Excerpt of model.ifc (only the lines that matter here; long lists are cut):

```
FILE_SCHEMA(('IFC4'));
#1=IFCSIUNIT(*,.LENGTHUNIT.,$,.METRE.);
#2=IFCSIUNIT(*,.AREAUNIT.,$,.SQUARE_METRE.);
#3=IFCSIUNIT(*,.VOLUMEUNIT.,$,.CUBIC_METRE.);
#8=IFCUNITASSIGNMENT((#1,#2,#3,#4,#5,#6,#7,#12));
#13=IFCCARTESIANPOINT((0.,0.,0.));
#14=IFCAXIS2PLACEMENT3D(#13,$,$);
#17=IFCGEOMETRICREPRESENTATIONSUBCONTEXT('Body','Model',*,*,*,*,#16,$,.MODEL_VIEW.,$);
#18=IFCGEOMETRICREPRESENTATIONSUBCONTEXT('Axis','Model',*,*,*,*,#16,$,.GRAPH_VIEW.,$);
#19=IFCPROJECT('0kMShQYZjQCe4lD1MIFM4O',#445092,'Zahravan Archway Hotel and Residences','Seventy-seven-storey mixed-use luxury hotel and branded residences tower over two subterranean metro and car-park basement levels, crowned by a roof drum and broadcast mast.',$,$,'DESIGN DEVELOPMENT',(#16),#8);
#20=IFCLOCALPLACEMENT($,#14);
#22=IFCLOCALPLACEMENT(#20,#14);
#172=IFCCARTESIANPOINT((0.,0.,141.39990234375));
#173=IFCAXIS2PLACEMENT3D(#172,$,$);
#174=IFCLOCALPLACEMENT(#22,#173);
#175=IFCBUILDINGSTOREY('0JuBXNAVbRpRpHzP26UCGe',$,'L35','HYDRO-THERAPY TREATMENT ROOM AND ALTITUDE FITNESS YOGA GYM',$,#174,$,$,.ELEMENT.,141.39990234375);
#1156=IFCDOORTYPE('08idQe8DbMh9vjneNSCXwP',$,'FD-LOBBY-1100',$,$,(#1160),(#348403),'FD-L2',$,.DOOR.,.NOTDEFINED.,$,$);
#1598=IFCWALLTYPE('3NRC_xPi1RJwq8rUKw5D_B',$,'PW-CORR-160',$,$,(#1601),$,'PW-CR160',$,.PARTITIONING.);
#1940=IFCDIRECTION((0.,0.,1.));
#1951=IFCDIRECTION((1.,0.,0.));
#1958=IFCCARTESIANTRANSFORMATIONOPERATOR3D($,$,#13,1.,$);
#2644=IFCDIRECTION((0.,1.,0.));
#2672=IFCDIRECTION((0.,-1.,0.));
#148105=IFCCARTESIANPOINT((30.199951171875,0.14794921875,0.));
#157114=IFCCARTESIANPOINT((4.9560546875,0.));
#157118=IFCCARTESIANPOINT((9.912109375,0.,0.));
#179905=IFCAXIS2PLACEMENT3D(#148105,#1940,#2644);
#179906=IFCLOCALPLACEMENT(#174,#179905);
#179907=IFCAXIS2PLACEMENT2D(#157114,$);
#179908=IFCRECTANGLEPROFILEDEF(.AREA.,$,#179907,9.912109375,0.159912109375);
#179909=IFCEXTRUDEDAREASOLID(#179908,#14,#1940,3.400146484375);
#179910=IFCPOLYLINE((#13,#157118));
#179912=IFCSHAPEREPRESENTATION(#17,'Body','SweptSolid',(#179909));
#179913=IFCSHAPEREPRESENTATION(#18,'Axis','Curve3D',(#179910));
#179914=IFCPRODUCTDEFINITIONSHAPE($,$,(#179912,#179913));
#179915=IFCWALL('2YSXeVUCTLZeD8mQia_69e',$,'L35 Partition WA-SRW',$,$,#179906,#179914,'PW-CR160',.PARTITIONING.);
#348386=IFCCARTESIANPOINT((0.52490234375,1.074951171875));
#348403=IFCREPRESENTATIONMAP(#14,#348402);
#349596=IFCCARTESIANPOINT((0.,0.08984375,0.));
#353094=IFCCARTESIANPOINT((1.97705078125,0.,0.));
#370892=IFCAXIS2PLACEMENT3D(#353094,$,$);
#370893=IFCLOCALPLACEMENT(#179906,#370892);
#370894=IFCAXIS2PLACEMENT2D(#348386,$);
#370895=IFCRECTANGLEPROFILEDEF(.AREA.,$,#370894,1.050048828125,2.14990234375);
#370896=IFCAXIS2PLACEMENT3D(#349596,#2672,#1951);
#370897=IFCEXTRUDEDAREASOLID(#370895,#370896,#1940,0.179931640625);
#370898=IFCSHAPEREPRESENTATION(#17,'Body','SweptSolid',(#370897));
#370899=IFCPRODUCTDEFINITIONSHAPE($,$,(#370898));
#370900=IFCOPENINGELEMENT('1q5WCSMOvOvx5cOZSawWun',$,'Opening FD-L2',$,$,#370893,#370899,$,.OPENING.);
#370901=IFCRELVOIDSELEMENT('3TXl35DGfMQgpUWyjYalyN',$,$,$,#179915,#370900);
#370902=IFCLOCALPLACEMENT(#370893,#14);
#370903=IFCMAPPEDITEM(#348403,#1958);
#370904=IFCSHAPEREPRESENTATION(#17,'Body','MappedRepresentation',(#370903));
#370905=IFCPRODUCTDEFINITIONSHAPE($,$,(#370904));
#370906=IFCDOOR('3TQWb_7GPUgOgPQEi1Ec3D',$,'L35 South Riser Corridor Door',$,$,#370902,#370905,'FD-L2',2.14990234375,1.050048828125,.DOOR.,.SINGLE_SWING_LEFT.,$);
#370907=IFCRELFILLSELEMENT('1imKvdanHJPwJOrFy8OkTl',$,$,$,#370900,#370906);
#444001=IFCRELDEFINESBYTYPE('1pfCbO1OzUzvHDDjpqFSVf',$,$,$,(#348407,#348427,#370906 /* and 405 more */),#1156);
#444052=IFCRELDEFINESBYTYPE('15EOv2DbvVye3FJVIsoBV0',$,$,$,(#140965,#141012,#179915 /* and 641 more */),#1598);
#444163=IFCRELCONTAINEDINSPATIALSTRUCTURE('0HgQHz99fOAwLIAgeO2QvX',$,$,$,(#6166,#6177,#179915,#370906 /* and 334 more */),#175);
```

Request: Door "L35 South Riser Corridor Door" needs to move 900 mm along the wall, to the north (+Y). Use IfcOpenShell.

```python
import ifcopenshell
import ifcopenshell.api.geometry
import ifcopenshell.util.placement
import ifcopenshell.util.unit

model = ifcopenshell.open("model.ifc")
unit_scale = ifcopenshell.util.unit.calculate_unit_scale(model)

door = model.by_guid("3TQWb_7GPUgOgPQEi1Ec3D")
opening = door.FillsVoids[0].RelatingOpeningElement
wall = opening.VoidsElements[0].RelatingBuildingElement

wall_matrix = ifcopenshell.util.placement.get_local_placement(wall.ObjectPlacement)
shift = wall_matrix[:3, 0] * 0.9 / unit_scale
before = ifcopenshell.util.placement.get_local_placement(door.ObjectPlacement)[:3, 3].copy()

# The door is placed relative to its opening, so it follows when the opening moves.
matrix = ifcopenshell.util.placement.get_local_placement(opening.ObjectPlacement)
matrix[:3, 3] += shift
ifcopenshell.api.geometry.edit_object_placement(
    model, product=opening, matrix=matrix, is_si=False, should_transform_children=True
)

after = ifcopenshell.util.placement.get_local_placement(door.ObjectPlacement)[:3, 3]
print("door moved by", (after - before).round(3) + 0.0)

model.write("model_rev.ifc")
```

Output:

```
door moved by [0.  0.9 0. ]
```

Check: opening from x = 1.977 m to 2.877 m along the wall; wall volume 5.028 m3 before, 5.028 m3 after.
